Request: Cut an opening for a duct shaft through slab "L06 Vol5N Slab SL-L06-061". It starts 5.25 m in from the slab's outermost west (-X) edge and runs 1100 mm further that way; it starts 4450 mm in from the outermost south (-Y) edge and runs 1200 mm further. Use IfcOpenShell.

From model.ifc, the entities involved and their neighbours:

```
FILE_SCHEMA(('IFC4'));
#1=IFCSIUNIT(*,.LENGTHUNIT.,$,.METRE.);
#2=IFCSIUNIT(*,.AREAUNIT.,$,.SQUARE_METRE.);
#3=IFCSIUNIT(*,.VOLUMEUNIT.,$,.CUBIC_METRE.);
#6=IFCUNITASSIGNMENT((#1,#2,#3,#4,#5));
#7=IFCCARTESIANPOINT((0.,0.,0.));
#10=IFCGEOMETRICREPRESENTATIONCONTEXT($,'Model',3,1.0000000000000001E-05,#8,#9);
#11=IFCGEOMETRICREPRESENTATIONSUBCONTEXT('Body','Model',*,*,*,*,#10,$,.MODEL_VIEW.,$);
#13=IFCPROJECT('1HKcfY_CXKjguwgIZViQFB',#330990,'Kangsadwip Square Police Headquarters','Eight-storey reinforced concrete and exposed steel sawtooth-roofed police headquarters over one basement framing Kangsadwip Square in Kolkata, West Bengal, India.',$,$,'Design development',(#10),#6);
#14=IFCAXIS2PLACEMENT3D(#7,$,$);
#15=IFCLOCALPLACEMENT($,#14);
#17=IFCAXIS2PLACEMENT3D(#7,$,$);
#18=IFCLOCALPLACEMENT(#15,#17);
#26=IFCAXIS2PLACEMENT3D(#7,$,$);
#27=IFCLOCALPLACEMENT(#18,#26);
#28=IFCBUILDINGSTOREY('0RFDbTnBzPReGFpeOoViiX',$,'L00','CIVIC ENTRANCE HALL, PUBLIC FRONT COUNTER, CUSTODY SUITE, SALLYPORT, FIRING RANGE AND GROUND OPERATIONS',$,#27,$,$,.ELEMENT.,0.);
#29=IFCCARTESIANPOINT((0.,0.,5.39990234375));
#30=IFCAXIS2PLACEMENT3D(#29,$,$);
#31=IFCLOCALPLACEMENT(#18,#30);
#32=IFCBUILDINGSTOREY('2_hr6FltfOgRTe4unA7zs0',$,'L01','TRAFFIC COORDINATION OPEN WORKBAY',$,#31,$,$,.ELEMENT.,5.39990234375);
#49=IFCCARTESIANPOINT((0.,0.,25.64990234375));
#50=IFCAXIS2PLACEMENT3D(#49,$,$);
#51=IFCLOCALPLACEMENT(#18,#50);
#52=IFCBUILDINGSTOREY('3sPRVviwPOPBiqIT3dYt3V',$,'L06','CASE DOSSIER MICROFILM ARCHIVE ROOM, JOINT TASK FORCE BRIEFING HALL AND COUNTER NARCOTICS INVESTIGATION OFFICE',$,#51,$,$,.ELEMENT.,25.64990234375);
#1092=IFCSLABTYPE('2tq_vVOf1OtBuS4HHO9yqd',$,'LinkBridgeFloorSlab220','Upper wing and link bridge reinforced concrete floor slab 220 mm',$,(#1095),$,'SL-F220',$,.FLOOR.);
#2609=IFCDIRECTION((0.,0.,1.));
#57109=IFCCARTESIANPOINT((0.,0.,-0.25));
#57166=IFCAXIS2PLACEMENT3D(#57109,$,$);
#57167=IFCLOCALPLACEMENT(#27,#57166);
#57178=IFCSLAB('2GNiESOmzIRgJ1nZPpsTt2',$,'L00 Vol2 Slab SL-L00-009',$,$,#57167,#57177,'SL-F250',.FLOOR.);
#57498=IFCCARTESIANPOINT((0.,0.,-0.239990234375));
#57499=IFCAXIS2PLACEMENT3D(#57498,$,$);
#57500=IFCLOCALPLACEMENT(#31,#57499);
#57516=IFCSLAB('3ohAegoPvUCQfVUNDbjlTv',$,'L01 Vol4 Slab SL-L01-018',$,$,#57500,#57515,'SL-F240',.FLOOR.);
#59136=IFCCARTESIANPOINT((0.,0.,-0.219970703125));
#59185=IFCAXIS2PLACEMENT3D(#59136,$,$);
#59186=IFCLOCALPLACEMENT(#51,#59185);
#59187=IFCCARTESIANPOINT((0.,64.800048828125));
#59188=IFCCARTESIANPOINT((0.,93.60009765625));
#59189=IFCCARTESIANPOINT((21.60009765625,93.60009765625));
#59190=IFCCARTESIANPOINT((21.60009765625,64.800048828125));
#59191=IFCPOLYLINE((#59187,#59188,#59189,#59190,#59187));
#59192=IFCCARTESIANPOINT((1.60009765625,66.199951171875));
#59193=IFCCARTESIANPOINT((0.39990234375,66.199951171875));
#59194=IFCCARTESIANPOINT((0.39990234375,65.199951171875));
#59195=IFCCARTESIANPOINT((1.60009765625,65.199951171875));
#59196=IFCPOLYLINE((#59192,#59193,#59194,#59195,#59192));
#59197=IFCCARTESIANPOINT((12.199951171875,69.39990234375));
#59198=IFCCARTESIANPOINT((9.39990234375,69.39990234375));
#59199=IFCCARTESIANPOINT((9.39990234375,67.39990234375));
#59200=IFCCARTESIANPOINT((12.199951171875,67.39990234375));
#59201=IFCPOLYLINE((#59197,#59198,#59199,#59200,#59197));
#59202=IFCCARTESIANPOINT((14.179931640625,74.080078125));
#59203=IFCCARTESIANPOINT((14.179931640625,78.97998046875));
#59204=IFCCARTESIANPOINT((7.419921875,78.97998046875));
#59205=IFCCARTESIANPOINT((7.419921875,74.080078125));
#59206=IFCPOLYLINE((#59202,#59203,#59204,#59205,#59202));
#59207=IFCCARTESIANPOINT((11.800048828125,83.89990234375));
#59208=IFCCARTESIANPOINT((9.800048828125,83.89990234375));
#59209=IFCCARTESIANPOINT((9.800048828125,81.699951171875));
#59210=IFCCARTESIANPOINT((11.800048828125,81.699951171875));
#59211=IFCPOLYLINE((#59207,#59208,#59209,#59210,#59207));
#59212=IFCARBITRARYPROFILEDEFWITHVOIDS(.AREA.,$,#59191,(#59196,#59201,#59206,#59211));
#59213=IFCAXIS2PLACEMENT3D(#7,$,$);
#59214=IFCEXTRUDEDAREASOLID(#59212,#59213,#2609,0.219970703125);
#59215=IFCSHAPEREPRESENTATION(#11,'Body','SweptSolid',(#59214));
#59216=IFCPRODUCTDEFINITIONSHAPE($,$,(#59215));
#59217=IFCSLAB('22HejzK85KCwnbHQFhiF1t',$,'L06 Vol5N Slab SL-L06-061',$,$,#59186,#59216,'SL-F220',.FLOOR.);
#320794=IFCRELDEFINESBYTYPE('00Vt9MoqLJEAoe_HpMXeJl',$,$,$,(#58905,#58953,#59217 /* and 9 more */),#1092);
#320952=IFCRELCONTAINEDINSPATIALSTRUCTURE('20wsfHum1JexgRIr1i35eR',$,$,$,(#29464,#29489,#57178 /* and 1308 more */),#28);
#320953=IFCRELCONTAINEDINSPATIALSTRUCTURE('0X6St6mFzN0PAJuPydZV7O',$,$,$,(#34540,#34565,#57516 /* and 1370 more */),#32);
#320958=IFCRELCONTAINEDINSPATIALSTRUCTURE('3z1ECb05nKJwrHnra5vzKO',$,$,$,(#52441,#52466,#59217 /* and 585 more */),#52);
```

```python
import numpy as np
import ifcopenshell
import ifcopenshell.api.feature
import ifcopenshell.api.geometry
import ifcopenshell.api.root
import ifcopenshell.geom
import ifcopenshell.util.placement
import ifcopenshell.util.representation
import ifcopenshell.util.shape
import ifcopenshell.util.unit

model = ifcopenshell.open("model.ifc")
unit_scale = ifcopenshell.util.unit.calculate_unit_scale(model)
settings = ifcopenshell.geom.settings()


def volume(element):
    """Net volume in cubic metres, openings subtracted."""
    shape = ifcopenshell.geom.create_shape(settings, element)
    return ifcopenshell.util.shape.get_volume(shape.geometry)


slab = model.by_id(59217)
before = volume(slab)

# Extent in the slab's own axes, in metres. The edges named are its -X and -Y sides.
slab_shape = ifcopenshell.geom.create_shape(settings, slab)
vertices = ifcopenshell.util.shape.get_vertices(slab_shape.geometry)
x_min, y_min, bottom = vertices.min(axis=0)
top = vertices[:, 2].max()

opening = ifcopenshell.api.root.create_entity(model, ifc_class="IfcOpeningElement", name="Duct shaft opening", predefined_type="OPENING")
context = ifcopenshell.util.representation.get_context(model, "Model", "Body", "MODEL_VIEW")
width, depth = 1.1, 1.2
outline = [(0.0, 0.0), (width, 0.0), (width, depth), (0.0, depth), (0.0, 0.0)]
# Overshoot both faces by 50 mm so the cut is clean.
shape = ifcopenshell.api.geometry.add_slab_representation(
    model, context=context, depth=top - bottom + 0.1, polyline=outline
)
ifcopenshell.api.geometry.assign_representation(model, product=opening, representation=shape)

matrix = ifcopenshell.util.placement.get_local_placement(slab.ObjectPlacement)
matrix[:, 3] = matrix @ np.append(np.array([x_min + 5.25, y_min + 4.45, bottom - 0.05]) / unit_scale, 1.0)
ifcopenshell.api.geometry.edit_object_placement(model, product=opening, matrix=matrix, is_si=False)
ifcopenshell.api.feature.add_feature(model, feature=opening, element=slab)

after = volume(slab)

print(f"slab volume {before:.3f} -> {after:.3f} m3")

model.write("model_v2.ifc")
```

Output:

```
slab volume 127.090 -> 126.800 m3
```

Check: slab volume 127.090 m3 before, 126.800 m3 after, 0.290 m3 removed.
